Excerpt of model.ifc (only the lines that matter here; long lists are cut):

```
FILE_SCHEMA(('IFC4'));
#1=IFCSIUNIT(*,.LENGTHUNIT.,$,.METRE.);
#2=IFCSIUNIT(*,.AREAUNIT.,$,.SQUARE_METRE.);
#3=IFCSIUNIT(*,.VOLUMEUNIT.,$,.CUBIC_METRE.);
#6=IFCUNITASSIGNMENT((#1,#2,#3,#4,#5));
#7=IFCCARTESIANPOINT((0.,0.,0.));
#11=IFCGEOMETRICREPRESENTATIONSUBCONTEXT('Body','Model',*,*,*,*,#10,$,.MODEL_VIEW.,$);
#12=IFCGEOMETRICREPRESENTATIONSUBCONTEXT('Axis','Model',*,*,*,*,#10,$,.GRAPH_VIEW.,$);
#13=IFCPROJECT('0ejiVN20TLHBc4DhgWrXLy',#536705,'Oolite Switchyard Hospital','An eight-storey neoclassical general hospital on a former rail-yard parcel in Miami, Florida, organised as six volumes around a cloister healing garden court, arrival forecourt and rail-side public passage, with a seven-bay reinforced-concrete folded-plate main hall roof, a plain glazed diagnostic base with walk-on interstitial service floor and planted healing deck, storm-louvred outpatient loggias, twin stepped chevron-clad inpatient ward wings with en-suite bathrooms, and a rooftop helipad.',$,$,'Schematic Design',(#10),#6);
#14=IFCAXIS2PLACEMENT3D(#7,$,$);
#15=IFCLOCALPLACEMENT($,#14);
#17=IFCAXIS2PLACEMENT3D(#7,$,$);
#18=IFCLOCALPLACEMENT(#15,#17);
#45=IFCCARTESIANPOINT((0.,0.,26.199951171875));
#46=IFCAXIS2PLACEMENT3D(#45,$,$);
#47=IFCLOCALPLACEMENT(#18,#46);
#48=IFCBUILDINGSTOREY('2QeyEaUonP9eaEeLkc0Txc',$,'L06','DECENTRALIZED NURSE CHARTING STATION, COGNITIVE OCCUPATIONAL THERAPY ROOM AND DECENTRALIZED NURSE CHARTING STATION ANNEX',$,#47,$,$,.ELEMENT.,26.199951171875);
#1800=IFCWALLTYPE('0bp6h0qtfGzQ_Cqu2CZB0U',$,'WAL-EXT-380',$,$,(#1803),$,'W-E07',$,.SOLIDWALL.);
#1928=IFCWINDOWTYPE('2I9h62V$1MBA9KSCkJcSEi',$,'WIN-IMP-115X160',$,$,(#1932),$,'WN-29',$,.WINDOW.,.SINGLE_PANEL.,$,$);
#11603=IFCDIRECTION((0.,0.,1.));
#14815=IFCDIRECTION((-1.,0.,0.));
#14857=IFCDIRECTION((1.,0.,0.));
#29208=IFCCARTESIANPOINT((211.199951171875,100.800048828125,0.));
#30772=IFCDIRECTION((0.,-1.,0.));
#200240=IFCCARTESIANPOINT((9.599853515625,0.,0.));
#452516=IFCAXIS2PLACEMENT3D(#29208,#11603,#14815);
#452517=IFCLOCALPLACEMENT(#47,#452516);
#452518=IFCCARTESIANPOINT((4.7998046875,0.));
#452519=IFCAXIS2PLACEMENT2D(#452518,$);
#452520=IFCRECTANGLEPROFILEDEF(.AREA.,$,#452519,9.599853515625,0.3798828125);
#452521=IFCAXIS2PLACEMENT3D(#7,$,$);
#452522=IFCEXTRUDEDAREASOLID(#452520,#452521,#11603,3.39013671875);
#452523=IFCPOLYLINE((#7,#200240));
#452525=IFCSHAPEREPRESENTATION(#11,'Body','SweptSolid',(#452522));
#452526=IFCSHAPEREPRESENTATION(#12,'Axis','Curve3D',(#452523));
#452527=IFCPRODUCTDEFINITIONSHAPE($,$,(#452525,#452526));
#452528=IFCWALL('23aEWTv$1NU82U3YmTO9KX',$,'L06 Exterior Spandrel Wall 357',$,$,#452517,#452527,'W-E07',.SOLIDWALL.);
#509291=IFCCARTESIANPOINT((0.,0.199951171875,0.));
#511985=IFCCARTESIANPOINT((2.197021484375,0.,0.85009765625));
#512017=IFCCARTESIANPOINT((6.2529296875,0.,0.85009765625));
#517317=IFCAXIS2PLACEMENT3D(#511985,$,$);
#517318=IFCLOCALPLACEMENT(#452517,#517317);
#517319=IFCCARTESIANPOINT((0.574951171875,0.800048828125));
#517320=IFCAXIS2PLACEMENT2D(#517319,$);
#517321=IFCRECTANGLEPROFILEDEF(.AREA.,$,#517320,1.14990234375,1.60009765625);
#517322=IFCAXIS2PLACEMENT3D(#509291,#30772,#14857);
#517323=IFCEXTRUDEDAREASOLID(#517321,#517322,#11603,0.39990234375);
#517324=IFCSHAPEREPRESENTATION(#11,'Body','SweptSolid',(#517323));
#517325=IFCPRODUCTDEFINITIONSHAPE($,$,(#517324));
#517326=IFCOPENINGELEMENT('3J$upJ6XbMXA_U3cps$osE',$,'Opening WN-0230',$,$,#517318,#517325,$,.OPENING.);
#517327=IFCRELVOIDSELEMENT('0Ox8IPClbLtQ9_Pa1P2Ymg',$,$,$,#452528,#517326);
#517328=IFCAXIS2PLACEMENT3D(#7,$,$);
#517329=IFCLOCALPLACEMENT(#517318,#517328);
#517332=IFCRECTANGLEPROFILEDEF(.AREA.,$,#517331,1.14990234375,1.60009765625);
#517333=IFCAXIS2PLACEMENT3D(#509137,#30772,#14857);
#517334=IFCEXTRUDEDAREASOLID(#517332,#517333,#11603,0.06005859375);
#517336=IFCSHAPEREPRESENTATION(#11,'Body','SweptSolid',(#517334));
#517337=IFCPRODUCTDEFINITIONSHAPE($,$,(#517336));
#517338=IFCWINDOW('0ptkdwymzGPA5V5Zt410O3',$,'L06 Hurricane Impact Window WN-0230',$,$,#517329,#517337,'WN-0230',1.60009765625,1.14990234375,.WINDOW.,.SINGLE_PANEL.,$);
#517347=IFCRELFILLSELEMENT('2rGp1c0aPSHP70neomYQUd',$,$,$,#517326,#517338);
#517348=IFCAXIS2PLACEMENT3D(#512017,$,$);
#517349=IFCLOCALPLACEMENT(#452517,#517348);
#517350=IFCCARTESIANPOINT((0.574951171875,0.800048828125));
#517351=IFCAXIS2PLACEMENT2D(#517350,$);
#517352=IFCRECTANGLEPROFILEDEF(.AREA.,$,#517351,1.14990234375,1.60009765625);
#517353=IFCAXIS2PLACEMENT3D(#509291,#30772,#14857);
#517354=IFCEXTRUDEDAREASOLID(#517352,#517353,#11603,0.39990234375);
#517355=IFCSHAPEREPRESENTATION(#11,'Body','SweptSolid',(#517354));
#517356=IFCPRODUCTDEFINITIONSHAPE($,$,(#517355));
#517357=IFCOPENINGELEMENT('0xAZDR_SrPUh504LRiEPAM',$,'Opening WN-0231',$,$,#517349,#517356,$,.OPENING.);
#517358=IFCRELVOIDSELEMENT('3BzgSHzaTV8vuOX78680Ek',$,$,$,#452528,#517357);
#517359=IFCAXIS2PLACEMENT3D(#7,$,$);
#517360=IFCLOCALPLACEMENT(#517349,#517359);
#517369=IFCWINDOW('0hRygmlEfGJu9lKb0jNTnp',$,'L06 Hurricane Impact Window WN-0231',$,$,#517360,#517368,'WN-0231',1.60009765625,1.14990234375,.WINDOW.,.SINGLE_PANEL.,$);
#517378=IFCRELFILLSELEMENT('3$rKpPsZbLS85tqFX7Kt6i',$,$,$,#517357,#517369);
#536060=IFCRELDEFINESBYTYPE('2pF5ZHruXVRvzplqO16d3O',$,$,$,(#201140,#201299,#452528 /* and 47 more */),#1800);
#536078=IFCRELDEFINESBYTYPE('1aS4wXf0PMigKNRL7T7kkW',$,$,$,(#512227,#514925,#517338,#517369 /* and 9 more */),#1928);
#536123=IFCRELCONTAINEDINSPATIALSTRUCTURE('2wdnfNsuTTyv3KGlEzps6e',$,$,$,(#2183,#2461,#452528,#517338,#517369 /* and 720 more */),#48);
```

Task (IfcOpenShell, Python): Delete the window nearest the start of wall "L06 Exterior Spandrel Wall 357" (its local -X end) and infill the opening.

```python
import ifcopenshell
import ifcopenshell.api.feature
import ifcopenshell.api.root
import ifcopenshell.geom
import ifcopenshell.util.shape

model = ifcopenshell.open("model.ifc")
settings = ifcopenshell.geom.settings()


def volume(element):
    """Net volume in cubic metres, openings subtracted."""
    shape = ifcopenshell.geom.create_shape(settings, element)
    return ifcopenshell.util.shape.get_volume(shape.geometry)


window = model.by_id(517338)
opening = window.FillsVoids[0].RelatingOpeningElement
wall = opening.VoidsElements[0].RelatingBuildingElement
before = volume(wall)

ifcopenshell.api.root.remove_product(model, product=window)
ifcopenshell.api.feature.remove_feature(model, feature=opening)

after = volume(wall)

print(f"wall volume {before:.3f} -> {after:.3f} m3")

model.write("model-out.ifc")
```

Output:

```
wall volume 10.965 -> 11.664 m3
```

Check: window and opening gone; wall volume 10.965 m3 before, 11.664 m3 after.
